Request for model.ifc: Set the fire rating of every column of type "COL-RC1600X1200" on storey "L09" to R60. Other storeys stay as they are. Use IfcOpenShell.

First a look at what the model holds.

```python
import ifcopenshell
import ifcopenshell.util.element

model = ifcopenshell.open("model.ifc")
print(model.schema)
storey = next(s for s in model.by_type("IfcBuildingStorey") if s.Name == "L09")
columns = [e for e in ifcopenshell.util.element.get_decomposition(storey) if e.is_a("IfcColumn")]
seen = {}
for e in columns:
    element_type = ifcopenshell.util.element.get_type(e)
    key = (element_type.Name if element_type != e and element_type else None, ifcopenshell.util.element.get_pset(e, "Pset_ColumnCommon", "FireRating"))
    seen[key] = seen.get(key, 0) + 1
for (name, value), count in sorted(seen.items(), key=str):
    print(count, "x", name, "|", value)
```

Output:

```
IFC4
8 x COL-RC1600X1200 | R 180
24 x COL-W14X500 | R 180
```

```python
import ifcopenshell
import ifcopenshell.api.pset
import ifcopenshell.util.element

model = ifcopenshell.open("model.ifc")

storey = next(s for s in model.by_type("IfcBuildingStorey") if s.Name == "L09")
columns = [e for e in ifcopenshell.util.element.get_decomposition(storey) if e.is_a("IfcColumn")]

count = 0
for e in columns:
    element_type = ifcopenshell.util.element.get_type(e)
    if element_type in (None, e) or element_type.Name != "COL-RC1600X1200":
        continue
    found = ifcopenshell.util.element.get_pset(e, "Pset_ColumnCommon", should_inherit=False)
    if found:
        pset = model.by_id(found["id"])
        if len(ifcopenshell.util.element.get_elements_by_pset(pset)) > 1:
            pset = ifcopenshell.api.pset.unshare_pset(model, products=[e], pset=pset)[0]
    else:
        pset = ifcopenshell.api.pset.add_pset(model, product=e, name="Pset_ColumnCommon")
    ifcopenshell.api.pset.edit_pset(model, pset=pset, properties={"FireRating": "R60"})
    count += 1

print(count, "columns updated")

model.write("model_v2.ifc")
```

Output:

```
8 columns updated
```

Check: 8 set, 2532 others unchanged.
